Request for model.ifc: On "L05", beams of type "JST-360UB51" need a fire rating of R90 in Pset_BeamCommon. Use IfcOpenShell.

First a look at what the model holds.

```python
import ifcopenshell
import ifcopenshell.util.element

model = ifcopenshell.open("model.ifc")
print(model.schema)
storey = next(s for s in model.by_type("IfcBuildingStorey") if s.Name == "L05")
beams = [e for e in ifcopenshell.util.element.get_decomposition(storey) if e.is_a("IfcBeam")]
seen = {}
for e in beams:
    element_type = ifcopenshell.util.element.get_type(e)
    key = (element_type.Name if element_type != e and element_type else None, ifcopenshell.util.element.get_pset(e, "Pset_BeamCommon", "FireRating"))
    seen[key] = seen.get(key, 0) + 1
for (name, value), count in sorted(seen.items(), key=str):
    print(count, "x", name, "|", value)
```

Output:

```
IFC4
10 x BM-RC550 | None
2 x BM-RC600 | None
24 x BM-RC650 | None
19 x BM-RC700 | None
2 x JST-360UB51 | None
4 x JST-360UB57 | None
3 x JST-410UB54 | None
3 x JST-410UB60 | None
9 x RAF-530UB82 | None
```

```python
import ifcopenshell
import ifcopenshell.api.pset
import ifcopenshell.util.element

model = ifcopenshell.open("model.ifc")

storey = next(s for s in model.by_type("IfcBuildingStorey") if s.Name == "L05")
beams = [e for e in ifcopenshell.util.element.get_decomposition(storey) if e.is_a("IfcBeam")]

count = 0
for e in beams:
    element_type = ifcopenshell.util.element.get_type(e)
    if element_type in (None, e) or element_type.Name != "JST-360UB51":
        continue
    # add_pset returns the element's existing set when there is one.
    pset = ifcopenshell.api.pset.add_pset(model, product=e, name="Pset_BeamCommon")
    ifcopenshell.api.pset.edit_pset(model, pset=pset, properties={"FireRating": "R90"})
    count += 1

print(count, "beams updated")

model.write("model_v2.ifc")
```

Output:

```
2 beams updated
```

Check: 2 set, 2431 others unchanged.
